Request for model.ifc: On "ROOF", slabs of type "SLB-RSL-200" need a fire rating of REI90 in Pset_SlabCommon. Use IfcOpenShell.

First a look at what the model holds.

```python
import ifcopenshell
import ifcopenshell.util.element

model = ifcopenshell.open("model.ifc")
print(model.schema)
storey = next(s for s in model.by_type("IfcBuildingStorey") if s.Name == "ROOF")
slabs = [e for e in ifcopenshell.util.element.get_decomposition(storey) if e.is_a("IfcSlab")]
seen = {}
for e in slabs:
    element_type = ifcopenshell.util.element.get_type(e)
    key = (element_type.Name if element_type != e and element_type else None, ifcopenshell.util.element.get_pset(e, "Pset_SlabCommon", "FireRating"))
    seen[key] = seen.get(key, 0) + 1
for (name, value), count in sorted(seen.items(), key=str):
    print(count, "x", name, "|", value)
```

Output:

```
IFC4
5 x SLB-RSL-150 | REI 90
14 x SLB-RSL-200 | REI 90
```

```python
import ifcopenshell
import ifcopenshell.api.pset
import ifcopenshell.util.element

model = ifcopenshell.open("model.ifc")

storey = next(s for s in model.by_type("IfcBuildingStorey") if s.Name == "ROOF")
slabs = [e for e in ifcopenshell.util.element.get_decomposition(storey) if e.is_a("IfcSlab")]

count = 0
for e in slabs:
    element_type = ifcopenshell.util.element.get_type(e)
    if element_type in (None, e) or element_type.Name != "SLB-RSL-200":
        continue
    # add_pset returns the element's existing set when there is one.
    pset = ifcopenshell.api.pset.add_pset(model, product=e, name="Pset_SlabCommon")
    ifcopenshell.api.pset.edit_pset(model, pset=pset, properties={"FireRating": "REI90"})
    count += 1

print(count, "slabs updated")

model.write("model_rev.ifc")
```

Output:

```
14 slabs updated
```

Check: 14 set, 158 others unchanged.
